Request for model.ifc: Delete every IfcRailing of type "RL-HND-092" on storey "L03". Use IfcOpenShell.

First a look at what the model holds.

```python
import ifcopenshell
import ifcopenshell.util.element

model = ifcopenshell.open("model.ifc")
print(model.schema)
storey = next(s for s in model.by_type("IfcBuildingStorey") if s.Name == "L03")
railings = [e for e in ifcopenshell.util.element.get_decomposition(storey) if e.is_a("IfcRailing")]
seen = {}
for e in railings:
    element_type = ifcopenshell.util.element.get_type(e)
    name = element_type.Name if element_type not in (None, e) else None
    seen[name] = seen.get(name, 0) + 1
for name, count in sorted(seen.items(), key=str):
    print(count, "x", name)
```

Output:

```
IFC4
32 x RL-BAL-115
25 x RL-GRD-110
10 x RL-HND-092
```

```python
import ifcopenshell
import ifcopenshell.api.root
import ifcopenshell.util.element

model = ifcopenshell.open("model.ifc")

storey = next(s for s in model.by_type("IfcBuildingStorey") if s.Name == "L03")
railings = [e for e in ifcopenshell.util.element.get_decomposition(storey) if e.is_a("IfcRailing")]
targets = [e for e in railings if (t := ifcopenshell.util.element.get_type(e)) not in (None, e) and t.Name == "RL-HND-092"]

for e in targets:
    ifcopenshell.api.root.remove_product(model, product=e)
print(len(targets), "removed")

model.write("model_edited.ifc")
```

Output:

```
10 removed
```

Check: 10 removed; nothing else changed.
